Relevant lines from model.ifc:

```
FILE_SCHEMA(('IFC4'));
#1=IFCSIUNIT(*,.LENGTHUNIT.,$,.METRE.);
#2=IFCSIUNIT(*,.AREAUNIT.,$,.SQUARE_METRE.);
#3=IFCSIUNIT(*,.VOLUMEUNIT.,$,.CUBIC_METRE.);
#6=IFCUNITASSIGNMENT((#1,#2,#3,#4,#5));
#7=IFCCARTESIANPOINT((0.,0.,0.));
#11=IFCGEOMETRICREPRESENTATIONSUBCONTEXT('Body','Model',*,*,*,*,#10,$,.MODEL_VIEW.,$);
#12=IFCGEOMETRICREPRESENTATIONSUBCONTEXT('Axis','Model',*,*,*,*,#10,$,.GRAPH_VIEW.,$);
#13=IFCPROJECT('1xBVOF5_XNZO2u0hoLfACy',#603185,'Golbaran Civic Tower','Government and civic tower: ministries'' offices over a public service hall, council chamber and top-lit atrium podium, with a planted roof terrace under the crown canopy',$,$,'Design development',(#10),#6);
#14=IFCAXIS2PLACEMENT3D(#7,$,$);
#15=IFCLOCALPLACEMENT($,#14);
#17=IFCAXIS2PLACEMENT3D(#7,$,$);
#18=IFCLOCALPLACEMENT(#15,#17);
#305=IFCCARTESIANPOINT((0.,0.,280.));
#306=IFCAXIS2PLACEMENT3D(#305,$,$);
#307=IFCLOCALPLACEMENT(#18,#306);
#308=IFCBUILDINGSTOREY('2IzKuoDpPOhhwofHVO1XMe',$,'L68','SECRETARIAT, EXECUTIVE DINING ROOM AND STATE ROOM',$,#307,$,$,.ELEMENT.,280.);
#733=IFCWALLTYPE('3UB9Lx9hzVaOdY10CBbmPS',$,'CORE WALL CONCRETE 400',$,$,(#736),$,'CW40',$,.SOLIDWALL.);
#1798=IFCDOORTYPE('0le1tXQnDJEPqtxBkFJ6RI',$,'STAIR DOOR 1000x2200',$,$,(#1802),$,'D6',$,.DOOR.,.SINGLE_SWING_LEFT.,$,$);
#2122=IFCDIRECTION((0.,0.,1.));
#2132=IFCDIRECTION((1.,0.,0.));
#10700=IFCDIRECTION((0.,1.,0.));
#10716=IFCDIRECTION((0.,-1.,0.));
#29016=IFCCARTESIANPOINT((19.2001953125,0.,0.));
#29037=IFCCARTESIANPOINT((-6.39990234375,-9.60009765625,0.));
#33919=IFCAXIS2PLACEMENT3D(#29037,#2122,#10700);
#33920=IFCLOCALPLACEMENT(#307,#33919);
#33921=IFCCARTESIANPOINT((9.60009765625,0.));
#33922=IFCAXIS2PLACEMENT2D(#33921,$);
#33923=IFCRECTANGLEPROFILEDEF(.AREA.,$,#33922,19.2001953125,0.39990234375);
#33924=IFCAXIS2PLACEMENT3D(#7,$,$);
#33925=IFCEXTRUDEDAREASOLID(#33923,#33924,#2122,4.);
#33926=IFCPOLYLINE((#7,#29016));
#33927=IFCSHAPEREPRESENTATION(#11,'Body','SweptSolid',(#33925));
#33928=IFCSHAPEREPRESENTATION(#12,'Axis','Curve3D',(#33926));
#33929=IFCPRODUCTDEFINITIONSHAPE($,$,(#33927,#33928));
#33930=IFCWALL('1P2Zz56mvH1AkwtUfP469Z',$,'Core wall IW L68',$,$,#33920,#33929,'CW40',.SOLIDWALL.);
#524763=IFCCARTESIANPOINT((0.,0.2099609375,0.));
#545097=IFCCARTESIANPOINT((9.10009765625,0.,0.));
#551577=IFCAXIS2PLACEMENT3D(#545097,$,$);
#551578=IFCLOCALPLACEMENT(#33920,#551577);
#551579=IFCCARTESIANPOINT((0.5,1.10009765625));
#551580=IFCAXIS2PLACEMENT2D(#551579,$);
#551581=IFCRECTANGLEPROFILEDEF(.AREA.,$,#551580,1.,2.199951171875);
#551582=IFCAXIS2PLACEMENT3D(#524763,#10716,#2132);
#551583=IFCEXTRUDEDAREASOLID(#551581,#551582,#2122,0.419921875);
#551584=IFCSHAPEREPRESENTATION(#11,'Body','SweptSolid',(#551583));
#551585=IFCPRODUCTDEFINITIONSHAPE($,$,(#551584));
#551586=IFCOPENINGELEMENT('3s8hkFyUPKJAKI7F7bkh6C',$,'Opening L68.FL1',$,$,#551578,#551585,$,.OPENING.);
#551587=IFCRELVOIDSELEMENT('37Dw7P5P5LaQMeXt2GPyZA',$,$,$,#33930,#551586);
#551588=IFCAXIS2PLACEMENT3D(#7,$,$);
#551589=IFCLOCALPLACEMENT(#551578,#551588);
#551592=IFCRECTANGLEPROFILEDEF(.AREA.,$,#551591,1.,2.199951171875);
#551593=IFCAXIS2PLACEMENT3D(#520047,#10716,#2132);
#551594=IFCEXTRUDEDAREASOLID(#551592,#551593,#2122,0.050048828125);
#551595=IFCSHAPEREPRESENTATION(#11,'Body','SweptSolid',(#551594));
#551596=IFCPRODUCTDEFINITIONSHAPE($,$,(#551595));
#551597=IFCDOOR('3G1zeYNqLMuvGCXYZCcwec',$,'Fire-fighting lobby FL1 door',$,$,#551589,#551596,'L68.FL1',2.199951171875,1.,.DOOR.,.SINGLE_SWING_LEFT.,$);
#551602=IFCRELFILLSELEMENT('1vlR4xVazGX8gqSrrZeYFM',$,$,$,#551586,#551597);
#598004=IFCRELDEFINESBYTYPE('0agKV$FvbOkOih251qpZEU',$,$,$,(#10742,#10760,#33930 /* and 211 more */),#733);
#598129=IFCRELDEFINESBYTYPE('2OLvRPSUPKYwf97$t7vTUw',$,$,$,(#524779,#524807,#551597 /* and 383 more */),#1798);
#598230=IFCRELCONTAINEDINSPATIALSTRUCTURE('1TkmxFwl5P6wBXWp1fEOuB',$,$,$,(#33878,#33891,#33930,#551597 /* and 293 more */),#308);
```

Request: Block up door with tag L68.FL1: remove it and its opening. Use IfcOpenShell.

```python
import ifcopenshell
import ifcopenshell.api.feature
import ifcopenshell.api.root
import ifcopenshell.geom
import ifcopenshell.util.shape

model = ifcopenshell.open("model.ifc")
settings = ifcopenshell.geom.settings()


def volume(element):
    """Net volume in cubic metres, openings subtracted."""
    shape = ifcopenshell.geom.create_shape(settings, element)
    return ifcopenshell.util.shape.get_volume(shape.geometry)


door = model.by_guid("3G1zeYNqLMuvGCXYZCcwec")
opening = door.FillsVoids[0].RelatingOpeningElement
wall = opening.VoidsElements[0].RelatingBuildingElement
before = volume(wall)

ifcopenshell.api.root.remove_product(model, product=door)
ifcopenshell.api.feature.remove_feature(model, feature=opening)

after = volume(wall)

print(f"wall volume {before:.3f} -> {after:.3f} m3")

model.write("model_edited.ifc")
```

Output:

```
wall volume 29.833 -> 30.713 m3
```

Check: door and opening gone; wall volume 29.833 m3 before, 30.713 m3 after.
